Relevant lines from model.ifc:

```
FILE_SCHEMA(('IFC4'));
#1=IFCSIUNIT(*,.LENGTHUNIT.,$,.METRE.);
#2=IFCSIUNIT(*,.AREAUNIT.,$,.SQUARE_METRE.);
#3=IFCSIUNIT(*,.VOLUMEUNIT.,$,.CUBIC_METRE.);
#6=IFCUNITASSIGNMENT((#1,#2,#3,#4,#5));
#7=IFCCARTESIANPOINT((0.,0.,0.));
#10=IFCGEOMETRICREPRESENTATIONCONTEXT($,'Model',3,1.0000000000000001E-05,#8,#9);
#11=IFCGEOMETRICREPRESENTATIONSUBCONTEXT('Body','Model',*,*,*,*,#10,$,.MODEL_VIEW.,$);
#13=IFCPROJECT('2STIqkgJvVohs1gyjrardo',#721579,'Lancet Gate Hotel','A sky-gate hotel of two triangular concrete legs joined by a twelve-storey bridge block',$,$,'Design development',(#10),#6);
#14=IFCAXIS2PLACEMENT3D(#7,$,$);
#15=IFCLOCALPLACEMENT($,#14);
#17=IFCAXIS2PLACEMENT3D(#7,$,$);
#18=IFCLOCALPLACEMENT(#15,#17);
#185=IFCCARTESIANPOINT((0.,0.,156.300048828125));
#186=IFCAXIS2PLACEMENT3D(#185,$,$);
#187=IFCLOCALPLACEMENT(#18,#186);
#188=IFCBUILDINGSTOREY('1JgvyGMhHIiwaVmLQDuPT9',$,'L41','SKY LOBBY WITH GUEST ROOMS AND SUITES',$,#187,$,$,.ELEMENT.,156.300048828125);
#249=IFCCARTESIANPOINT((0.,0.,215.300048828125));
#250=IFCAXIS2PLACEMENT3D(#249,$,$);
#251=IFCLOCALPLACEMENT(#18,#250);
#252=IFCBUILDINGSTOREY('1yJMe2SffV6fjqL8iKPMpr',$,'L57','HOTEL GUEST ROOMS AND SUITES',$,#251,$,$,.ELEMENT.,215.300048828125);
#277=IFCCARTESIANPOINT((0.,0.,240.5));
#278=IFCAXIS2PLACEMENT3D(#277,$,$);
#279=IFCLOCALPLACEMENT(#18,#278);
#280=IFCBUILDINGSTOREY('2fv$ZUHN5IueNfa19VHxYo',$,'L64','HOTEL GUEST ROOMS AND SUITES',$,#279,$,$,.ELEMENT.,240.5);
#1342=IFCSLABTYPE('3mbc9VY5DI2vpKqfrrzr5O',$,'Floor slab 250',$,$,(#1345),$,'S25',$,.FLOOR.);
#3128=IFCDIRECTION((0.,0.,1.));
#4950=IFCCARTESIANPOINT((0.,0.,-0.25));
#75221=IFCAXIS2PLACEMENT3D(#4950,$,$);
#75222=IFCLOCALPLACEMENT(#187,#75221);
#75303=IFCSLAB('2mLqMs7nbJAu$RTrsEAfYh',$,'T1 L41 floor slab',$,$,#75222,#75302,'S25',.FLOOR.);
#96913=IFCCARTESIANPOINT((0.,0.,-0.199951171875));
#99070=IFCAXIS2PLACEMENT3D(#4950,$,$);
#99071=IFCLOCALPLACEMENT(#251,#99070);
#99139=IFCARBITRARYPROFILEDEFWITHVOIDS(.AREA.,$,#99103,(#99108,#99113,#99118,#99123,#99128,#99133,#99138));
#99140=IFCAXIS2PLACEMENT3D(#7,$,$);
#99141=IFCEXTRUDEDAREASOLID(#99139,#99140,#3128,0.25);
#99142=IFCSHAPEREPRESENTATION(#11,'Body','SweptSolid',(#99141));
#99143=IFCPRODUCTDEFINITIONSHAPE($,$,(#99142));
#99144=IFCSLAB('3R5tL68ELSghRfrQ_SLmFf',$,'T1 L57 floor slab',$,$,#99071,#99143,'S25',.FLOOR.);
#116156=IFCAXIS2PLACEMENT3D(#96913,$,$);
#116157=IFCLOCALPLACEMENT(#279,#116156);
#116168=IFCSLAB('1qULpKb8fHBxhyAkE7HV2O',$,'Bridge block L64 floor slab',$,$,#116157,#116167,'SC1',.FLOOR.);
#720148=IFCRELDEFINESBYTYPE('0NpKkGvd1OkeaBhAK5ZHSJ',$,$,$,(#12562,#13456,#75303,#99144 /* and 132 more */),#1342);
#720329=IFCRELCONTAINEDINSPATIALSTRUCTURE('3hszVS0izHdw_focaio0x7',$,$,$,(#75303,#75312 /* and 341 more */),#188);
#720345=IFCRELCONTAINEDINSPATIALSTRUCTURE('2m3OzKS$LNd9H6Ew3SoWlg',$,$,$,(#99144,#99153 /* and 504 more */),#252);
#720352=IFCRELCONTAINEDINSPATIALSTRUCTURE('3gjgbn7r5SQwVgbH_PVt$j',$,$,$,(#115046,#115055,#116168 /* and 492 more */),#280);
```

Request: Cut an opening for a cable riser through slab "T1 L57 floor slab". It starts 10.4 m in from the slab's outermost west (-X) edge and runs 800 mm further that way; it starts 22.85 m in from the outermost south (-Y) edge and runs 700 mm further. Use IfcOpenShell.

```python
import numpy as np
import ifcopenshell
import ifcopenshell.api.feature
import ifcopenshell.api.geometry
import ifcopenshell.api.root
import ifcopenshell.geom
import ifcopenshell.util.placement
import ifcopenshell.util.representation
import ifcopenshell.util.shape
import ifcopenshell.util.unit

model = ifcopenshell.open("model.ifc")
unit_scale = ifcopenshell.util.unit.calculate_unit_scale(model)
settings = ifcopenshell.geom.settings()


def volume(element):
    """Net volume in cubic metres, openings subtracted."""
    shape = ifcopenshell.geom.create_shape(settings, element)
    return ifcopenshell.util.shape.get_volume(shape.geometry)


slab = model.by_id(99144)
before = volume(slab)

# Extent in the slab's own axes, in metres. The edges named are its -X and -Y sides.
slab_shape = ifcopenshell.geom.create_shape(settings, slab)
vertices = ifcopenshell.util.shape.get_vertices(slab_shape.geometry)
x_min, y_min, bottom = vertices.min(axis=0)
top = vertices[:, 2].max()

opening = ifcopenshell.api.root.create_entity(model, ifc_class="IfcOpeningElement", name="Cable riser opening", predefined_type="OPENING")
context = ifcopenshell.util.representation.get_context(model, "Model", "Body", "MODEL_VIEW")
width, depth = 0.8, 0.7
outline = [(0.0, 0.0), (width, 0.0), (width, depth), (0.0, depth), (0.0, 0.0)]
# Overshoot both faces by 50 mm so the cut is clean.
shape = ifcopenshell.api.geometry.add_slab_representation(
    model, context=context, depth=top - bottom + 0.1, polyline=outline
)
ifcopenshell.api.geometry.assign_representation(model, product=opening, representation=shape)

matrix = ifcopenshell.util.placement.get_local_placement(slab.ObjectPlacement)
matrix[:, 3] = matrix @ np.append(np.array([x_min + 10.4, y_min + 22.85, bottom - 0.05]) / unit_scale, 1.0)
ifcopenshell.api.geometry.edit_object_placement(model, product=opening, matrix=matrix, is_si=False)
ifcopenshell.api.feature.add_feature(model, feature=opening, element=slab)

after = volume(slab)

print(f"slab volume {before:.3f} -> {after:.3f} m3")

model.write("model_edited.ifc")
```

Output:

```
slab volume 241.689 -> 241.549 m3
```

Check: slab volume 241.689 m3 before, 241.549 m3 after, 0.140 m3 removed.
